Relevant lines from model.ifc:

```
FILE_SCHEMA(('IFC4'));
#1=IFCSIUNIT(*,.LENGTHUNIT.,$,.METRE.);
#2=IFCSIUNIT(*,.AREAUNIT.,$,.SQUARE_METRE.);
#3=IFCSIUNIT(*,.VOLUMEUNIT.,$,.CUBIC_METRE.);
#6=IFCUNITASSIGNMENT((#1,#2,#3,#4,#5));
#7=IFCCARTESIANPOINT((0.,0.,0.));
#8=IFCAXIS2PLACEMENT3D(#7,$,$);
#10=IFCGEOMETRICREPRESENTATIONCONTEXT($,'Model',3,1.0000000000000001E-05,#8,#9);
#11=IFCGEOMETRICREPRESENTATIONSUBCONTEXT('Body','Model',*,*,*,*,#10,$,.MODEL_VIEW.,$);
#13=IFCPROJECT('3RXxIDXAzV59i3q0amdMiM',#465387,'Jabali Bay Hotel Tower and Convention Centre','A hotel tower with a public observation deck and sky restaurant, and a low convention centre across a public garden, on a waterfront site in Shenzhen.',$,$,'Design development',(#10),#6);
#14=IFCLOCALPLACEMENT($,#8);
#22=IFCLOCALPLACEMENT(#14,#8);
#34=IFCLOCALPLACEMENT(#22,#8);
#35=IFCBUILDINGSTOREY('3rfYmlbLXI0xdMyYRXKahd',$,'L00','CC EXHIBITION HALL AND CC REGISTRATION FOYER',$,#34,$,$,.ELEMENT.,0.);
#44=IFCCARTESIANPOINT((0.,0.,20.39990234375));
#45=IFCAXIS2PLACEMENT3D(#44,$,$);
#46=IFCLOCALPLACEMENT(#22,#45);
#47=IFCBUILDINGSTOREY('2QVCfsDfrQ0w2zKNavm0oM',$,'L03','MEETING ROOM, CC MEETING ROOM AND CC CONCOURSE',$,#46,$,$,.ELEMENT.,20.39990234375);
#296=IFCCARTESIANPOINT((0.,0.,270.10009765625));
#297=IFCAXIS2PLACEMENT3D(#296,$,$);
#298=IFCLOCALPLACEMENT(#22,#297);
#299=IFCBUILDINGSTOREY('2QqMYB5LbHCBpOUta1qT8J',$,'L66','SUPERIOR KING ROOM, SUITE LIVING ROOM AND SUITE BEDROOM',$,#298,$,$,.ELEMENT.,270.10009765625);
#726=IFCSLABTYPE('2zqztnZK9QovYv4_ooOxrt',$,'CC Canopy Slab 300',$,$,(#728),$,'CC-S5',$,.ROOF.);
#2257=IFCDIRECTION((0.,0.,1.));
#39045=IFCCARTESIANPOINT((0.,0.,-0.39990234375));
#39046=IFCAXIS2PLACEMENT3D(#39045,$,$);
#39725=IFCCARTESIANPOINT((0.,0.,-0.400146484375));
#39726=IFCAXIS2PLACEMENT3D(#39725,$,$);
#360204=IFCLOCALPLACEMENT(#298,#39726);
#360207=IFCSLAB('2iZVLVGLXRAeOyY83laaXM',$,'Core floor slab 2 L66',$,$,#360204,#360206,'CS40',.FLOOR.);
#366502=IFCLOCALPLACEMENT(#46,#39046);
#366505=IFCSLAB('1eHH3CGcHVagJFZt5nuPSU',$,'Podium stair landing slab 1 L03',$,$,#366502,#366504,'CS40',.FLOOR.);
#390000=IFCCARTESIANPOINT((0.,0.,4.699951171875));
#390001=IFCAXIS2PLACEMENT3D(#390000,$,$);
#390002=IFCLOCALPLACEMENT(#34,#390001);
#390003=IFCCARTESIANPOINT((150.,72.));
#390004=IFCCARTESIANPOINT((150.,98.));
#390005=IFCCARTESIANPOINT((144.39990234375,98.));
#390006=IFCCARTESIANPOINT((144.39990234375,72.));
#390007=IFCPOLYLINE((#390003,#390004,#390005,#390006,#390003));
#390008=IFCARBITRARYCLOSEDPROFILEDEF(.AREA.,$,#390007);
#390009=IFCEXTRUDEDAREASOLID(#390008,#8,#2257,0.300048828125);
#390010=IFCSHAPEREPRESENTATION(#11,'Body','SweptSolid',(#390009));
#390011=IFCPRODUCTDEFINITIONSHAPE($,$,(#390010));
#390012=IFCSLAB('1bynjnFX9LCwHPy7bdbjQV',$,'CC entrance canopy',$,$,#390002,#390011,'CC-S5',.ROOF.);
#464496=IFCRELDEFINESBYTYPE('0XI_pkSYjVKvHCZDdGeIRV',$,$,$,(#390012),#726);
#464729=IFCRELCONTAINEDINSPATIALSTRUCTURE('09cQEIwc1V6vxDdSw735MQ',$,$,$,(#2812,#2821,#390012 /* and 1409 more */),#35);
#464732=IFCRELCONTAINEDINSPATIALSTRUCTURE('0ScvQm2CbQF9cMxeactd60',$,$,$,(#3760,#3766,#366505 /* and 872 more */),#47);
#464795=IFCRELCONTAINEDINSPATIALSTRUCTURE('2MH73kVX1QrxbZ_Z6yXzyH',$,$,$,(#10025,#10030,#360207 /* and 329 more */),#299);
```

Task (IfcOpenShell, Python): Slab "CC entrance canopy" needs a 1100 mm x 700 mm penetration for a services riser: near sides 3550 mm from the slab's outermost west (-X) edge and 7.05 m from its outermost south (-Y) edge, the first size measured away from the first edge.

```python
import numpy as np
import ifcopenshell
import ifcopenshell.api.feature
import ifcopenshell.api.geometry
import ifcopenshell.api.root
import ifcopenshell.geom
import ifcopenshell.util.placement
import ifcopenshell.util.representation
import ifcopenshell.util.shape
import ifcopenshell.util.unit

model = ifcopenshell.open("model.ifc")
unit_scale = ifcopenshell.util.unit.calculate_unit_scale(model)
settings = ifcopenshell.geom.settings()


def volume(element):
    """Net volume in cubic metres, openings subtracted."""
    shape = ifcopenshell.geom.create_shape(settings, element)
    return ifcopenshell.util.shape.get_volume(shape.geometry)


slab = model.by_guid("1bynjnFX9LCwHPy7bdbjQV")
before = volume(slab)

# Extent in the slab's own axes, in metres. The edges named are its -X and -Y sides.
slab_shape = ifcopenshell.geom.create_shape(settings, slab)
vertices = ifcopenshell.util.shape.get_vertices(slab_shape.geometry)
x_min, y_min, bottom = vertices.min(axis=0)
top = vertices[:, 2].max()

opening = ifcopenshell.api.root.create_entity(model, ifc_class="IfcOpeningElement", name="Services riser opening", predefined_type="OPENING")
context = ifcopenshell.util.representation.get_context(model, "Model", "Body", "MODEL_VIEW")
width, depth = 1.1, 0.7
outline = [(0.0, 0.0), (width, 0.0), (width, depth), (0.0, depth), (0.0, 0.0)]
# Overshoot both faces by 50 mm so the cut is clean.
shape = ifcopenshell.api.geometry.add_slab_representation(
    model, context=context, depth=top - bottom + 0.1, polyline=outline
)
ifcopenshell.api.geometry.assign_representation(model, product=opening, representation=shape)

matrix = ifcopenshell.util.placement.get_local_placement(slab.ObjectPlacement)
matrix[:, 3] = matrix @ np.append(np.array([x_min + 3.55, y_min + 7.05, bottom - 0.05]) / unit_scale, 1.0)
ifcopenshell.api.geometry.edit_object_placement(model, product=opening, matrix=matrix, is_si=False)
ifcopenshell.api.feature.add_feature(model, feature=opening, element=slab)

after = volume(slab)

print(f"slab volume {before:.3f} -> {after:.3f} m3")

model.write("model_rev.ifc")
```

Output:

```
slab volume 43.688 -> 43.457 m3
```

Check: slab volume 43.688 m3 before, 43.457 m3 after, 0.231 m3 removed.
